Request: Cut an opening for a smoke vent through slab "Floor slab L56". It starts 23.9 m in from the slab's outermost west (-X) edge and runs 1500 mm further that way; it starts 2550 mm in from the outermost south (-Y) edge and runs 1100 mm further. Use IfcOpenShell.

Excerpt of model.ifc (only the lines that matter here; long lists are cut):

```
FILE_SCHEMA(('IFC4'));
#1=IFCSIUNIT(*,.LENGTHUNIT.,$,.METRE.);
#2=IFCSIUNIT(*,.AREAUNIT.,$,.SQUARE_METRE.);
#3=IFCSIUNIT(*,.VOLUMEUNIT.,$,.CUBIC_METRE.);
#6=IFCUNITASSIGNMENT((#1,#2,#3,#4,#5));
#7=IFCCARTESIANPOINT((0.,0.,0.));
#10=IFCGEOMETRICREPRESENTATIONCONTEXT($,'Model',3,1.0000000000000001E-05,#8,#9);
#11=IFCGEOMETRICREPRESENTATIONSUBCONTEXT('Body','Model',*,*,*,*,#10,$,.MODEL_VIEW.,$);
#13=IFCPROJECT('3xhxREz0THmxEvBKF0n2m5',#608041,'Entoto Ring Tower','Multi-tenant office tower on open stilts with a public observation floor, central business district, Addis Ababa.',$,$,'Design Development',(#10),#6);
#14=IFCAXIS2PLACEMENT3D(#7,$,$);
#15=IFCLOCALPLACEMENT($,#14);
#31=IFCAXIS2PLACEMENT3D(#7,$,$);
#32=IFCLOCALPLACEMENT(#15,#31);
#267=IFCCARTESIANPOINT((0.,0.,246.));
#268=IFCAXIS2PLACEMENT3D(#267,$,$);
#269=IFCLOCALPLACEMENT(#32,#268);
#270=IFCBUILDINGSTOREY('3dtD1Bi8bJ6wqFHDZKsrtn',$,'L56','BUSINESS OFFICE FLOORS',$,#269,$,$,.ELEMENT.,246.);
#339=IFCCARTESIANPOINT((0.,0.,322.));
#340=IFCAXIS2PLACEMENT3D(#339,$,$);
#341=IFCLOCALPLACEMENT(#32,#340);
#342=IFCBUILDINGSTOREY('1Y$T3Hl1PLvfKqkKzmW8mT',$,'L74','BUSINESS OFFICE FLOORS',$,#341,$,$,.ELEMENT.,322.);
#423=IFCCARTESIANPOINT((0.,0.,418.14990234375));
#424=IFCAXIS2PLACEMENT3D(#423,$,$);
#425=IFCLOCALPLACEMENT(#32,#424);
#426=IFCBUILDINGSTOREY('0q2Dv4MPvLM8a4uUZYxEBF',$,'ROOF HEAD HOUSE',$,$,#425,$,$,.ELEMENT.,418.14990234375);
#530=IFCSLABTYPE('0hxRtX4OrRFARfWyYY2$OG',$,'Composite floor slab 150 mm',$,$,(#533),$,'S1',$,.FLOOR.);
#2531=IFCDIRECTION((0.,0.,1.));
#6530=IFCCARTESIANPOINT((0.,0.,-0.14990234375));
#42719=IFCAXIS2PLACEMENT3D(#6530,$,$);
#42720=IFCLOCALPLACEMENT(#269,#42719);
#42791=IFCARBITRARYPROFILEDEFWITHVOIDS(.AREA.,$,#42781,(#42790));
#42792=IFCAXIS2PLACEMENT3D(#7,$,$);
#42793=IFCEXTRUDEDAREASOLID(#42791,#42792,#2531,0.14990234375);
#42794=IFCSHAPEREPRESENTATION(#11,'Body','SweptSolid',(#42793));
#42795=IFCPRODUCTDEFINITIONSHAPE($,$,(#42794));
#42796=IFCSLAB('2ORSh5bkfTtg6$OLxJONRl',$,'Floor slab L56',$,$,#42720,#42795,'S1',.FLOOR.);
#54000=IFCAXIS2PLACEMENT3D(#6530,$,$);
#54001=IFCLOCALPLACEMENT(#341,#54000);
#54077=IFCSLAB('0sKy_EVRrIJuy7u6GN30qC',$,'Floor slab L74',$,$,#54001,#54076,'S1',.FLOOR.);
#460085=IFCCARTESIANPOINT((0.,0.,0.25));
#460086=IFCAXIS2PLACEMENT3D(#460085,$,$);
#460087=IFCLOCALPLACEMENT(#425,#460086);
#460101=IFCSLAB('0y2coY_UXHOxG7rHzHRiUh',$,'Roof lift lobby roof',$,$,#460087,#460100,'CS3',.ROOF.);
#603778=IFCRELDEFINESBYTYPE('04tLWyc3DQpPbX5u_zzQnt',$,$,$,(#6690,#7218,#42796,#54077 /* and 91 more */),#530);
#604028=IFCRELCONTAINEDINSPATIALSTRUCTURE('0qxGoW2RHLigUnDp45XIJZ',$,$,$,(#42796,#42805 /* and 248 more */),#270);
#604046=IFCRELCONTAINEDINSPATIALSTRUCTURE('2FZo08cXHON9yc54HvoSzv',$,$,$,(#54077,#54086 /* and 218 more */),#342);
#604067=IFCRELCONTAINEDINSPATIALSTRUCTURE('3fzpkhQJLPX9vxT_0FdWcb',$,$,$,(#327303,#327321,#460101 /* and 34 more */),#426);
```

```python
import numpy as np
import ifcopenshell
import ifcopenshell.api.feature
import ifcopenshell.api.geometry
import ifcopenshell.api.root
import ifcopenshell.geom
import ifcopenshell.util.placement
import ifcopenshell.util.representation
import ifcopenshell.util.shape
import ifcopenshell.util.unit

model = ifcopenshell.open("model.ifc")
unit_scale = ifcopenshell.util.unit.calculate_unit_scale(model)
settings = ifcopenshell.geom.settings()


def volume(element):
    """Net volume in cubic metres, openings subtracted."""
    shape = ifcopenshell.geom.create_shape(settings, element)
    return ifcopenshell.util.shape.get_volume(shape.geometry)


slab = model.by_guid("2ORSh5bkfTtg6$OLxJONRl")
before = volume(slab)

# Extent in the slab's own axes, in metres. The edges named are its -X and -Y sides.
slab_shape = ifcopenshell.geom.create_shape(settings, slab)
vertices = ifcopenshell.util.shape.get_vertices(slab_shape.geometry)
x_min, y_min, bottom = vertices.min(axis=0)
top = vertices[:, 2].max()

opening = ifcopenshell.api.root.create_entity(model, ifc_class="IfcOpeningElement", name="Smoke vent opening", predefined_type="OPENING")
context = ifcopenshell.util.representation.get_context(model, "Model", "Body", "MODEL_VIEW")
width, depth = 1.5, 1.1
outline = [(0.0, 0.0), (width, 0.0), (width, depth), (0.0, depth), (0.0, 0.0)]
# Overshoot both faces by 50 mm so the cut is clean.
shape = ifcopenshell.api.geometry.add_slab_representation(
    model, context=context, depth=top - bottom + 0.1, polyline=outline
)
ifcopenshell.api.geometry.assign_representation(model, product=opening, representation=shape)

matrix = ifcopenshell.util.placement.get_local_placement(slab.ObjectPlacement)
matrix[:, 3] = matrix @ np.append(np.array([x_min + 23.9, y_min + 2.55, bottom - 0.05]) / unit_scale, 1.0)
ifcopenshell.api.geometry.edit_object_placement(model, product=opening, matrix=matrix, is_si=False)
ifcopenshell.api.feature.add_feature(model, feature=opening, element=slab)

after = volume(slab)

print(f"slab volume {before:.3f} -> {after:.3f} m3")

model.write("model_edited.ifc")
```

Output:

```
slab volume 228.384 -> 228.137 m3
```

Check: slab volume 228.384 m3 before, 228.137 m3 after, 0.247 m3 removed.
